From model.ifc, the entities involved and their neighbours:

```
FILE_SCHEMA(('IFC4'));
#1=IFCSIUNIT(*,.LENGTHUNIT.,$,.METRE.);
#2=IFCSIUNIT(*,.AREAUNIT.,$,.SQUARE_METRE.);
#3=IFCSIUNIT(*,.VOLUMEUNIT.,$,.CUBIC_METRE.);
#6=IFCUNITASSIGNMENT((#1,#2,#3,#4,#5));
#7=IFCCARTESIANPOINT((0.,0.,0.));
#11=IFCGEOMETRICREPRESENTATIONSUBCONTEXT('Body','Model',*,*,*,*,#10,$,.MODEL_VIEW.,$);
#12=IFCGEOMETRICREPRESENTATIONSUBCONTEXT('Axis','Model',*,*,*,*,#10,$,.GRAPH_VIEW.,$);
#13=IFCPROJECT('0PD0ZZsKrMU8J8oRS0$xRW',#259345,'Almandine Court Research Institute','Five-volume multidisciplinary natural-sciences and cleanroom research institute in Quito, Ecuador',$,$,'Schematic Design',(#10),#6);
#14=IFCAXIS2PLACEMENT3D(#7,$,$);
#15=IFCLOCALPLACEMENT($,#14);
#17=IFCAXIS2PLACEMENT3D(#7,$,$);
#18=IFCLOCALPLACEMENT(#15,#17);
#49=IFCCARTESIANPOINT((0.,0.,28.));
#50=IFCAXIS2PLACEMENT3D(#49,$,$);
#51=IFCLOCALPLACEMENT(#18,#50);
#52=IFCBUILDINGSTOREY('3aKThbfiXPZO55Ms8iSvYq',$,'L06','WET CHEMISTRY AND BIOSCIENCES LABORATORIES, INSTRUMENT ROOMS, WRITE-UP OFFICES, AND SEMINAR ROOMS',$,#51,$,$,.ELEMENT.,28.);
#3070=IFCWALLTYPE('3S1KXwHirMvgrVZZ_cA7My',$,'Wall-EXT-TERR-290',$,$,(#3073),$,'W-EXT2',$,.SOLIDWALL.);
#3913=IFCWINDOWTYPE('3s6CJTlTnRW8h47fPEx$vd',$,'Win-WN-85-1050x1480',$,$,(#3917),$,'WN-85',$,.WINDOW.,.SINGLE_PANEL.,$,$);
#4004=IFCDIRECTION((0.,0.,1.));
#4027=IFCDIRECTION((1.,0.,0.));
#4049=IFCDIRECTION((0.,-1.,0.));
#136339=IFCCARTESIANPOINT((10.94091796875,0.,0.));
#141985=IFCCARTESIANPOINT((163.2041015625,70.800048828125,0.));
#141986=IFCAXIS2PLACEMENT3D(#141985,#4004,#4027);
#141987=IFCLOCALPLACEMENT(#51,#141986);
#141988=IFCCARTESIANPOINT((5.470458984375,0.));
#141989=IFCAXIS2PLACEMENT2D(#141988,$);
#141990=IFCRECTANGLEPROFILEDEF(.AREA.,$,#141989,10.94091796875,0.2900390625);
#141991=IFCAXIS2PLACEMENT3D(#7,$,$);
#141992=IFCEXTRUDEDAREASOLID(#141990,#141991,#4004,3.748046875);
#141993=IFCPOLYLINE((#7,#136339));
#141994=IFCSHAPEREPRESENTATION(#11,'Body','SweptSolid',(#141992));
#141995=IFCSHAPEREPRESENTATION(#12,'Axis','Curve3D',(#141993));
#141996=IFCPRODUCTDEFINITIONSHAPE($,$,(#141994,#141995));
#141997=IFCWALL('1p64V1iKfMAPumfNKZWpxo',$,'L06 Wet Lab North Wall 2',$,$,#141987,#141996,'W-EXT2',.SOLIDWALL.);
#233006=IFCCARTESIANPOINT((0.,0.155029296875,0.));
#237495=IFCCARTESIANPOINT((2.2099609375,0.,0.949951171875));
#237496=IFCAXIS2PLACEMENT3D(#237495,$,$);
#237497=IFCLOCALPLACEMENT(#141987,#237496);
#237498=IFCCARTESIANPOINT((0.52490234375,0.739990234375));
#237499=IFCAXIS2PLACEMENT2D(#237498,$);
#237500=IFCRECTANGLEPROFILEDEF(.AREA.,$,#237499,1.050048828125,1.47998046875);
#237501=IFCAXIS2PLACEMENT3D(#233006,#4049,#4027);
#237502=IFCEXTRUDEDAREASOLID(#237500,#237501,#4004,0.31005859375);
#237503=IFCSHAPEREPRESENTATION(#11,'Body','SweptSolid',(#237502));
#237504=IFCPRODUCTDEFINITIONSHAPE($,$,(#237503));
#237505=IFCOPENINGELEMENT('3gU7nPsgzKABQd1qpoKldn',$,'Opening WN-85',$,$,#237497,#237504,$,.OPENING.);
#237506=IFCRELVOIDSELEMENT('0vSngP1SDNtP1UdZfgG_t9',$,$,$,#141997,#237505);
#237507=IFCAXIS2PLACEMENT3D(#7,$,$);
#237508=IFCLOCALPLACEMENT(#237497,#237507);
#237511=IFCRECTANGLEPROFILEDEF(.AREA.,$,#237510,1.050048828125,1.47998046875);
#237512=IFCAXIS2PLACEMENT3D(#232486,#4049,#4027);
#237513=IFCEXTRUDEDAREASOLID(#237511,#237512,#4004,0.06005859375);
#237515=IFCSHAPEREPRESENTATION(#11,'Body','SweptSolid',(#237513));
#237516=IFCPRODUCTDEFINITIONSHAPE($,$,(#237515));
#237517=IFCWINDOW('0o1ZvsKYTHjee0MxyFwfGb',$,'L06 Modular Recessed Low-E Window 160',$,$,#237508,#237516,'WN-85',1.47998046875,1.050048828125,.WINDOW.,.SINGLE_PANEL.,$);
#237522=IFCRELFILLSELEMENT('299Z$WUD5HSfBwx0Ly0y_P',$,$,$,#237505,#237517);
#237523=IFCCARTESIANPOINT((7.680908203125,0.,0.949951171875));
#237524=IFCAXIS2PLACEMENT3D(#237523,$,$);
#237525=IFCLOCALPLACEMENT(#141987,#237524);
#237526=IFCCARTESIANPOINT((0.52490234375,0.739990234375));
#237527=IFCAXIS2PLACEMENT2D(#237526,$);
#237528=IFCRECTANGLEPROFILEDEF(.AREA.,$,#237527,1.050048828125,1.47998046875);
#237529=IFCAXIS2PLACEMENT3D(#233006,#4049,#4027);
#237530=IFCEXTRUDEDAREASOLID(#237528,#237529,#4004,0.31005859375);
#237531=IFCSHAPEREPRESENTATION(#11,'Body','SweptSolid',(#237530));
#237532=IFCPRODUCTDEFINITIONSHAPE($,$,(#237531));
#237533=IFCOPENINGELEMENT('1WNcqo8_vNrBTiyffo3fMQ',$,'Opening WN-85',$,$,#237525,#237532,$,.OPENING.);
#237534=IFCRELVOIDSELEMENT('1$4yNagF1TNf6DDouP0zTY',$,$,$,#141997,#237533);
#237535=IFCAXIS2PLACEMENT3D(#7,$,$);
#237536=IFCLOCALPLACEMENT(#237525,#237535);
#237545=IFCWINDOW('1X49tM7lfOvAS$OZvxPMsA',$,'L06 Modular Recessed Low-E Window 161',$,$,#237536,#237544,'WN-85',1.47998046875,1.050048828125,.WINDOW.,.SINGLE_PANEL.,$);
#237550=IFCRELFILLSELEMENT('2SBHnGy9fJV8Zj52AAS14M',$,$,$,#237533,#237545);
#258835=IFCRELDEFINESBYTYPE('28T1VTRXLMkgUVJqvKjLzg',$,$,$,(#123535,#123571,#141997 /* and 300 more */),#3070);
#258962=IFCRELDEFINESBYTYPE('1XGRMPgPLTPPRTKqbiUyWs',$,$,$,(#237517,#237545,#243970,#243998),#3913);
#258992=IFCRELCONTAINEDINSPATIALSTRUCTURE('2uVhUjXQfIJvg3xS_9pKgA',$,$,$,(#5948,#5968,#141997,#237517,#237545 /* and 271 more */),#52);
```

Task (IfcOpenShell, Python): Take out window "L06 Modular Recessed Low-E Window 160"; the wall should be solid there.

```python
import ifcopenshell
import ifcopenshell.api.feature
import ifcopenshell.api.root
import ifcopenshell.geom
import ifcopenshell.util.shape

model = ifcopenshell.open("model.ifc")
settings = ifcopenshell.geom.settings()


def volume(element):
    """Net volume in cubic metres, openings subtracted."""
    shape = ifcopenshell.geom.create_shape(settings, element)
    return ifcopenshell.util.shape.get_volume(shape.geometry)


window = model.by_guid("0o1ZvsKYTHjee0MxyFwfGb")
opening = window.FillsVoids[0].RelatingOpeningElement
wall = opening.VoidsElements[0].RelatingBuildingElement
before = volume(wall)

ifcopenshell.api.root.remove_product(model, product=window)
ifcopenshell.api.feature.remove_feature(model, feature=opening)

after = volume(wall)

print(f"wall volume {before:.3f} -> {after:.3f} m3")

model.write("model_updated.ifc")
```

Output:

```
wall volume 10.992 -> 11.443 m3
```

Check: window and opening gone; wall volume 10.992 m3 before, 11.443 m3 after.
